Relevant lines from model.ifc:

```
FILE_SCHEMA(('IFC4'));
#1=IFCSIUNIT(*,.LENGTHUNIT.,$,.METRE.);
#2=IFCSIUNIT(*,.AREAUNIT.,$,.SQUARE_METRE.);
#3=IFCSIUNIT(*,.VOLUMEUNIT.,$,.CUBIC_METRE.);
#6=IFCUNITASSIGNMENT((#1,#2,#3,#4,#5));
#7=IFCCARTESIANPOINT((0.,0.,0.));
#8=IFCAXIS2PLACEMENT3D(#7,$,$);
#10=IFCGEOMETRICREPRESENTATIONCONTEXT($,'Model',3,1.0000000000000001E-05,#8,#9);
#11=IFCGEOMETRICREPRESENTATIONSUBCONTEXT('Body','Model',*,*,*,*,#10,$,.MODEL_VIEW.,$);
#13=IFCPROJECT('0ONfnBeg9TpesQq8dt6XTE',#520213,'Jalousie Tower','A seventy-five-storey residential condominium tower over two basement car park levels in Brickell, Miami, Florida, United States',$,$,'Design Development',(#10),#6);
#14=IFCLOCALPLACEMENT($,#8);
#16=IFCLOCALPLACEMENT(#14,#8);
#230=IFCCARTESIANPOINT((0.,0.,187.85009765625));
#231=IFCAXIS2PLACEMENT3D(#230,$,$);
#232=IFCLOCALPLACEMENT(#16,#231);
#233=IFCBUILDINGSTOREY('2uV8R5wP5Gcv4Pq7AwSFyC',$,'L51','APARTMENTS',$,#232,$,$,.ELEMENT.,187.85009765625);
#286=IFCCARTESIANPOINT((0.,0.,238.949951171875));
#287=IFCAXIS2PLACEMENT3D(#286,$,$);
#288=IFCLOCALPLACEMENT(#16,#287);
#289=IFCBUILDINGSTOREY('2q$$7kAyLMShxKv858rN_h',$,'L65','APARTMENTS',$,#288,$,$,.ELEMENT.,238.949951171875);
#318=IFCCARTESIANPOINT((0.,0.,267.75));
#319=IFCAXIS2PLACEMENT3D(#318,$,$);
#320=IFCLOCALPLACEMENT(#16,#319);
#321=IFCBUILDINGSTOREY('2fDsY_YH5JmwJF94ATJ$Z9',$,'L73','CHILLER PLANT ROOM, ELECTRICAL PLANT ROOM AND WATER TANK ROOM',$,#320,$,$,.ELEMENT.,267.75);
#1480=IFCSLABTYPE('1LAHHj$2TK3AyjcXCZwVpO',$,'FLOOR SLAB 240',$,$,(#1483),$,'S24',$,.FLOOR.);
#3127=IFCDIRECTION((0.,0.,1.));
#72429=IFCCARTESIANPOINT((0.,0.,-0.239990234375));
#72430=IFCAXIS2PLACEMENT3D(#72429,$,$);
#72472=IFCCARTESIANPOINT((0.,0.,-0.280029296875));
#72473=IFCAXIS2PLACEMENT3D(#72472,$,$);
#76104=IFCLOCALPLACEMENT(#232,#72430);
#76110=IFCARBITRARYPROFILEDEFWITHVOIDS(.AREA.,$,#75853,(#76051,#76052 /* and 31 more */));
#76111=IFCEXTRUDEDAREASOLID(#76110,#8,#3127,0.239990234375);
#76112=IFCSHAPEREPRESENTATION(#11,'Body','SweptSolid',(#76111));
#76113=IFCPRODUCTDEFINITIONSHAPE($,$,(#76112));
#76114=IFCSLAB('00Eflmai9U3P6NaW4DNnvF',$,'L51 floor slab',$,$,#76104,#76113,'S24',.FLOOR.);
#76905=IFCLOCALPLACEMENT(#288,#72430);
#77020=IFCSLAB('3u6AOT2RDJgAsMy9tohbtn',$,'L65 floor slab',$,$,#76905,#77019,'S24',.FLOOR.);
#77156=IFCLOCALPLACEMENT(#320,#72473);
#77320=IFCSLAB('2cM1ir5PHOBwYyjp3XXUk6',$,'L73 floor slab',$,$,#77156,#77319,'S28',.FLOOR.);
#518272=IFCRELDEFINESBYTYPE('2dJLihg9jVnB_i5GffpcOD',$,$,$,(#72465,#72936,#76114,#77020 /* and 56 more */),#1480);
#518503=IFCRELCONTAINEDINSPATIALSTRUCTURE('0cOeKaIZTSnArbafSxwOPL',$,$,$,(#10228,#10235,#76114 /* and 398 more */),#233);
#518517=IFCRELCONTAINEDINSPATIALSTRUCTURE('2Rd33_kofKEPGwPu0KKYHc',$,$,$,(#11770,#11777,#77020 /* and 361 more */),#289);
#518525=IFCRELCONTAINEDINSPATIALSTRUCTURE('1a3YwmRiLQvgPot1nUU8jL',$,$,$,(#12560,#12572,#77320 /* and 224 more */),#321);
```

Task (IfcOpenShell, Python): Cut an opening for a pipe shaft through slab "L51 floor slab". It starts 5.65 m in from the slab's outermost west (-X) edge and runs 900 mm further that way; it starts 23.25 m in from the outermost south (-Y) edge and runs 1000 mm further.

```python
import numpy as np
import ifcopenshell
import ifcopenshell.api.feature
import ifcopenshell.api.geometry
import ifcopenshell.api.root
import ifcopenshell.geom
import ifcopenshell.util.placement
import ifcopenshell.util.representation
import ifcopenshell.util.shape
import ifcopenshell.util.unit

model = ifcopenshell.open("model.ifc")
unit_scale = ifcopenshell.util.unit.calculate_unit_scale(model)
settings = ifcopenshell.geom.settings()


def volume(element):
    """Net volume in cubic metres, openings subtracted."""
    shape = ifcopenshell.geom.create_shape(settings, element)
    return ifcopenshell.util.shape.get_volume(shape.geometry)


slab = model.by_guid("00Eflmai9U3P6NaW4DNnvF")
before = volume(slab)

# Extent in the slab's own axes, in metres. The edges named are its -X and -Y sides.
slab_shape = ifcopenshell.geom.create_shape(settings, slab)
vertices = ifcopenshell.util.shape.get_vertices(slab_shape.geometry)
x_min, y_min, bottom = vertices.min(axis=0)
top = vertices[:, 2].max()

opening = ifcopenshell.api.root.create_entity(model, ifc_class="IfcOpeningElement", name="Pipe shaft opening", predefined_type="OPENING")
context = ifcopenshell.util.representation.get_context(model, "Model", "Body", "MODEL_VIEW")
width, depth = 0.9, 1
outline = [(0.0, 0.0), (width, 0.0), (width, depth), (0.0, depth), (0.0, 0.0)]
# Overshoot both faces by 50 mm so the cut is clean.
shape = ifcopenshell.api.geometry.add_slab_representation(
    model, context=context, depth=top - bottom + 0.1, polyline=outline
)
ifcopenshell.api.geometry.assign_representation(model, product=opening, representation=shape)

matrix = ifcopenshell.util.placement.get_local_placement(slab.ObjectPlacement)
matrix[:, 3] = matrix @ np.append(np.array([x_min + 5.65, y_min + 23.25, bottom - 0.05]) / unit_scale, 1.0)
ifcopenshell.api.geometry.edit_object_placement(model, product=opening, matrix=matrix, is_si=False)
ifcopenshell.api.feature.add_feature(model, feature=opening, element=slab)

after = volume(slab)

print(f"slab volume {before:.3f} -> {after:.3f} m3")

model.write("model_edited.ifc")
```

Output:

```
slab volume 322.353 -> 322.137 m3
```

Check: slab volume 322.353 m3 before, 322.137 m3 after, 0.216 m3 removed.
